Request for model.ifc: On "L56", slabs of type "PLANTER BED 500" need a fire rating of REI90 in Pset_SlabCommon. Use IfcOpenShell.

First a look at what the model holds.

```python
import ifcopenshell
import ifcopenshell.util.element

model = ifcopenshell.open("model.ifc")
print(model.schema)
storey = next(s for s in model.by_type("IfcBuildingStorey") if s.Name == "L56")
slabs = [e for e in ifcopenshell.util.element.get_decomposition(storey) if e.is_a("IfcSlab")]
seen = {}
for e in slabs:
    element_type = ifcopenshell.util.element.get_type(e)
    key = (element_type.Name if element_type != e and element_type else None, ifcopenshell.util.element.get_pset(e, "Pset_SlabCommon", "FireRating"))
    seen[key] = seen.get(key, 0) + 1
for (name, value), count in sorted(seen.items(), key=str):
    print(count, "x", name, "|", value)
```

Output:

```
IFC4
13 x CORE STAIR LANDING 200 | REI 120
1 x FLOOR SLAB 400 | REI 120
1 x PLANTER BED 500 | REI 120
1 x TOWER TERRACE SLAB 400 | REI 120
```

```python
import ifcopenshell
import ifcopenshell.api.pset
import ifcopenshell.util.element

model = ifcopenshell.open("model.ifc")

storey = next(s for s in model.by_type("IfcBuildingStorey") if s.Name == "L56")
slabs = [e for e in ifcopenshell.util.element.get_decomposition(storey) if e.is_a("IfcSlab")]

count = 0
for e in slabs:
    element_type = ifcopenshell.util.element.get_type(e)
    if element_type in (None, e) or element_type.Name != "PLANTER BED 500":
        continue
    found = ifcopenshell.util.element.get_pset(e, "Pset_SlabCommon", should_inherit=False)
    if found:
        pset = model.by_id(found["id"])
        if len(ifcopenshell.util.element.get_elements_by_pset(pset)) > 1:
            pset = ifcopenshell.api.pset.unshare_pset(model, products=[e], pset=pset)[0]
    else:
        pset = ifcopenshell.api.pset.add_pset(model, product=e, name="Pset_SlabCommon")
    ifcopenshell.api.pset.edit_pset(model, pset=pset, properties={"FireRating": "REI90"})
    count += 1

print(count, "slabs updated")

model.write("model_rev.ifc")
```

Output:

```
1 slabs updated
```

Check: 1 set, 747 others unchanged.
